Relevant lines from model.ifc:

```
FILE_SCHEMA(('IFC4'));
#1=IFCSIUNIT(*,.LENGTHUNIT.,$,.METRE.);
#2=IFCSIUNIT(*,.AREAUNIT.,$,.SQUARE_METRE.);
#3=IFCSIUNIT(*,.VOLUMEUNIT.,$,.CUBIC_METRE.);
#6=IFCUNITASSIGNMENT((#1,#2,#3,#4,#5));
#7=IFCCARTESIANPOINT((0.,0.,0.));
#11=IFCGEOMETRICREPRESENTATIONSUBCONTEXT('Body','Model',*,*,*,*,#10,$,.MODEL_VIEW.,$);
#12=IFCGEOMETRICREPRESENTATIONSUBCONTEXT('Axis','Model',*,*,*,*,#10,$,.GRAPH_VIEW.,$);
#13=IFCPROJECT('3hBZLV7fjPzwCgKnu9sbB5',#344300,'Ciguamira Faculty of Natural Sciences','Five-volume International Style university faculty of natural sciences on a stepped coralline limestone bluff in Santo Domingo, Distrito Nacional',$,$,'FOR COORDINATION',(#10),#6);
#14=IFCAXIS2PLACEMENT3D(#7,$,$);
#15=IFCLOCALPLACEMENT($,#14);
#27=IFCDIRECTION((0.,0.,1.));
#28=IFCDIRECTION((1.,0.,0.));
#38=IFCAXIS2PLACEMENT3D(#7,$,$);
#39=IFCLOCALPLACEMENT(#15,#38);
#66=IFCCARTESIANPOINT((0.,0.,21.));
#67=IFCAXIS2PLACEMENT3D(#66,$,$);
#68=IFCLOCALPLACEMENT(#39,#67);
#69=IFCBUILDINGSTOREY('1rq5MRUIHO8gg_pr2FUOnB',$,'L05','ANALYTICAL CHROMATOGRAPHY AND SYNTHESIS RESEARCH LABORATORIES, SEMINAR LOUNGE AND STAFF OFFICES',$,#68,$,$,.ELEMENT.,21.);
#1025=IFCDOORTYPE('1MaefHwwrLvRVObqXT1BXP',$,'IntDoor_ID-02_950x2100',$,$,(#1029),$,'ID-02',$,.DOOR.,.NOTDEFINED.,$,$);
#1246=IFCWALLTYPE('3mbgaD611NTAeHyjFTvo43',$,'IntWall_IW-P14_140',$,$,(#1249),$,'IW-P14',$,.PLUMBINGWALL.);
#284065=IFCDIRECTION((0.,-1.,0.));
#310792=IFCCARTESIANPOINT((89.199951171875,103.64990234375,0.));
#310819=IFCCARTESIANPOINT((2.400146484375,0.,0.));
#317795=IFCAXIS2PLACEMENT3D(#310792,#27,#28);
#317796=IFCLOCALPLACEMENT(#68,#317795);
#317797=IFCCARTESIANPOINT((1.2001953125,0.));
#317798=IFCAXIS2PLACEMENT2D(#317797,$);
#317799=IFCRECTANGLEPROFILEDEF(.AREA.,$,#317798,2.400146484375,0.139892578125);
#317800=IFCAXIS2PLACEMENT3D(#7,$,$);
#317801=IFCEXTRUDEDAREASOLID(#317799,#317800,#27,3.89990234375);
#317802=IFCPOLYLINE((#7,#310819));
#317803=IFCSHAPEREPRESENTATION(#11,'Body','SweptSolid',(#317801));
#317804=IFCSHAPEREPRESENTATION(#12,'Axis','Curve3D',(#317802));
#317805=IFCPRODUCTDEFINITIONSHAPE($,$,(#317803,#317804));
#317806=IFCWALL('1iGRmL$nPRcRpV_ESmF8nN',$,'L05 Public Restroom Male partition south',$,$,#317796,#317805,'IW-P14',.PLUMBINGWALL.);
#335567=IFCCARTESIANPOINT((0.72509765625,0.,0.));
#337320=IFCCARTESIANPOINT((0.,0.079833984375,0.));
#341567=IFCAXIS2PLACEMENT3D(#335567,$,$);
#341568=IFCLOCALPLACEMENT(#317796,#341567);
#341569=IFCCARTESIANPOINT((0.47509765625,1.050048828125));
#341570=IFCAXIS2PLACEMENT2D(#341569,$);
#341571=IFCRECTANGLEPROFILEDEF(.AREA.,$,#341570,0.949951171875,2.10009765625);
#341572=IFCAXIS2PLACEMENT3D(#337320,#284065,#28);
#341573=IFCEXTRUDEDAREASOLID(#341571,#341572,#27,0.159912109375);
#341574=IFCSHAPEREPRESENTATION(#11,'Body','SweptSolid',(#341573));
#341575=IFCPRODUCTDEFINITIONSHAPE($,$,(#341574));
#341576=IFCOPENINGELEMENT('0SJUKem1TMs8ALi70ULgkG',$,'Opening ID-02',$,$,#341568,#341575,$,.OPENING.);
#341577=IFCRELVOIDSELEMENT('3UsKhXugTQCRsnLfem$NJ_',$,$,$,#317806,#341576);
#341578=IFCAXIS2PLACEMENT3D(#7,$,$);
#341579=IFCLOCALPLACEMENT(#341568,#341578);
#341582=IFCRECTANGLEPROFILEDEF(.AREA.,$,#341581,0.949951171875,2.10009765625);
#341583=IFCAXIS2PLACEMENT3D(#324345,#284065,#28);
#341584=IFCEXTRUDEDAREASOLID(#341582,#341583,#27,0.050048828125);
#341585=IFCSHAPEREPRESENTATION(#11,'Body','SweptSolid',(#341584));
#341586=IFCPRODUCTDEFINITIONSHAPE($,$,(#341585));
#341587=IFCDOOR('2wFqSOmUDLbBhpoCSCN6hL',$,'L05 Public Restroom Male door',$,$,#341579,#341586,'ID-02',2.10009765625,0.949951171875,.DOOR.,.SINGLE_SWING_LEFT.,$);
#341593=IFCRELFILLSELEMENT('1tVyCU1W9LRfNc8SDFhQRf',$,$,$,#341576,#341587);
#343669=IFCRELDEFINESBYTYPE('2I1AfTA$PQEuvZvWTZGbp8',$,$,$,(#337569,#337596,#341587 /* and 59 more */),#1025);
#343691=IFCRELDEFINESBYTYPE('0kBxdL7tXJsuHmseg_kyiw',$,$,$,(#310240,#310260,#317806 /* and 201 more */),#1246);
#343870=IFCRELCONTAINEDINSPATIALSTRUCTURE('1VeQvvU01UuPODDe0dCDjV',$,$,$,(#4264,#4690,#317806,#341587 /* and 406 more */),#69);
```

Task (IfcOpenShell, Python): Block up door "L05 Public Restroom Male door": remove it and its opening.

```python
import ifcopenshell
import ifcopenshell.api.feature
import ifcopenshell.api.root
import ifcopenshell.geom
import ifcopenshell.util.shape

model = ifcopenshell.open("model.ifc")
settings = ifcopenshell.geom.settings()


def volume(element):
    """Net volume in cubic metres, openings subtracted."""
    shape = ifcopenshell.geom.create_shape(settings, element)
    return ifcopenshell.util.shape.get_volume(shape.geometry)


door = model.by_guid("2wFqSOmUDLbBhpoCSCN6hL")
opening = door.FillsVoids[0].RelatingOpeningElement
wall = opening.VoidsElements[0].RelatingBuildingElement
before = volume(wall)

ifcopenshell.api.root.remove_product(model, product=door)
ifcopenshell.api.feature.remove_feature(model, feature=opening)

after = volume(wall)

print(f"wall volume {before:.3f} -> {after:.3f} m3")

model.write("model_rev.ifc")
```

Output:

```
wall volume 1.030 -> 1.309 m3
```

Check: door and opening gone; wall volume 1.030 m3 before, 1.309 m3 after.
